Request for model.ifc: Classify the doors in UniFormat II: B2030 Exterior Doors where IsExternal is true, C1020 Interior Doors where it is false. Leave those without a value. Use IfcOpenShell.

First a look at what the model holds.

```python
import ifcopenshell
import ifcopenshell.util.element

model = ifcopenshell.open("model.ifc")
print(model.schema)
print("classifications:", [c.Name for c in model.by_type("IfcClassification")])
values = [ifcopenshell.util.element.get_pset(e, "Pset_DoorCommon", "IsExternal") for e in model.by_type("IfcDoor")]
for value in (True, False, None):
    print("IsExternal", value, values.count(value))
```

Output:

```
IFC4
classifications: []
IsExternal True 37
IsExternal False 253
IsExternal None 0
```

```python
import ifcopenshell
import ifcopenshell.api.classification
import ifcopenshell.util.element

model = ifcopenshell.open("model.ifc")

system = ifcopenshell.api.classification.add_classification(model, classification="UniFormat II")

doors = model.by_type("IfcDoor")
external = {e: ifcopenshell.util.element.get_pset(e, "Pset_DoorCommon", "IsExternal") for e in doors}
for flag, code, name in ((True, "B2030", "Exterior Doors"), (False, "C1020", "Interior Doors")):
    products = [e for e in doors if external[e] is flag]
    ifcopenshell.api.classification.add_reference(
        model, products=products, classification=system, identification=code, name=name
    )
    print(code, len(products))

model.write("model_edited.ifc")
```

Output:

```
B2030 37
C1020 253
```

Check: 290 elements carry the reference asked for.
